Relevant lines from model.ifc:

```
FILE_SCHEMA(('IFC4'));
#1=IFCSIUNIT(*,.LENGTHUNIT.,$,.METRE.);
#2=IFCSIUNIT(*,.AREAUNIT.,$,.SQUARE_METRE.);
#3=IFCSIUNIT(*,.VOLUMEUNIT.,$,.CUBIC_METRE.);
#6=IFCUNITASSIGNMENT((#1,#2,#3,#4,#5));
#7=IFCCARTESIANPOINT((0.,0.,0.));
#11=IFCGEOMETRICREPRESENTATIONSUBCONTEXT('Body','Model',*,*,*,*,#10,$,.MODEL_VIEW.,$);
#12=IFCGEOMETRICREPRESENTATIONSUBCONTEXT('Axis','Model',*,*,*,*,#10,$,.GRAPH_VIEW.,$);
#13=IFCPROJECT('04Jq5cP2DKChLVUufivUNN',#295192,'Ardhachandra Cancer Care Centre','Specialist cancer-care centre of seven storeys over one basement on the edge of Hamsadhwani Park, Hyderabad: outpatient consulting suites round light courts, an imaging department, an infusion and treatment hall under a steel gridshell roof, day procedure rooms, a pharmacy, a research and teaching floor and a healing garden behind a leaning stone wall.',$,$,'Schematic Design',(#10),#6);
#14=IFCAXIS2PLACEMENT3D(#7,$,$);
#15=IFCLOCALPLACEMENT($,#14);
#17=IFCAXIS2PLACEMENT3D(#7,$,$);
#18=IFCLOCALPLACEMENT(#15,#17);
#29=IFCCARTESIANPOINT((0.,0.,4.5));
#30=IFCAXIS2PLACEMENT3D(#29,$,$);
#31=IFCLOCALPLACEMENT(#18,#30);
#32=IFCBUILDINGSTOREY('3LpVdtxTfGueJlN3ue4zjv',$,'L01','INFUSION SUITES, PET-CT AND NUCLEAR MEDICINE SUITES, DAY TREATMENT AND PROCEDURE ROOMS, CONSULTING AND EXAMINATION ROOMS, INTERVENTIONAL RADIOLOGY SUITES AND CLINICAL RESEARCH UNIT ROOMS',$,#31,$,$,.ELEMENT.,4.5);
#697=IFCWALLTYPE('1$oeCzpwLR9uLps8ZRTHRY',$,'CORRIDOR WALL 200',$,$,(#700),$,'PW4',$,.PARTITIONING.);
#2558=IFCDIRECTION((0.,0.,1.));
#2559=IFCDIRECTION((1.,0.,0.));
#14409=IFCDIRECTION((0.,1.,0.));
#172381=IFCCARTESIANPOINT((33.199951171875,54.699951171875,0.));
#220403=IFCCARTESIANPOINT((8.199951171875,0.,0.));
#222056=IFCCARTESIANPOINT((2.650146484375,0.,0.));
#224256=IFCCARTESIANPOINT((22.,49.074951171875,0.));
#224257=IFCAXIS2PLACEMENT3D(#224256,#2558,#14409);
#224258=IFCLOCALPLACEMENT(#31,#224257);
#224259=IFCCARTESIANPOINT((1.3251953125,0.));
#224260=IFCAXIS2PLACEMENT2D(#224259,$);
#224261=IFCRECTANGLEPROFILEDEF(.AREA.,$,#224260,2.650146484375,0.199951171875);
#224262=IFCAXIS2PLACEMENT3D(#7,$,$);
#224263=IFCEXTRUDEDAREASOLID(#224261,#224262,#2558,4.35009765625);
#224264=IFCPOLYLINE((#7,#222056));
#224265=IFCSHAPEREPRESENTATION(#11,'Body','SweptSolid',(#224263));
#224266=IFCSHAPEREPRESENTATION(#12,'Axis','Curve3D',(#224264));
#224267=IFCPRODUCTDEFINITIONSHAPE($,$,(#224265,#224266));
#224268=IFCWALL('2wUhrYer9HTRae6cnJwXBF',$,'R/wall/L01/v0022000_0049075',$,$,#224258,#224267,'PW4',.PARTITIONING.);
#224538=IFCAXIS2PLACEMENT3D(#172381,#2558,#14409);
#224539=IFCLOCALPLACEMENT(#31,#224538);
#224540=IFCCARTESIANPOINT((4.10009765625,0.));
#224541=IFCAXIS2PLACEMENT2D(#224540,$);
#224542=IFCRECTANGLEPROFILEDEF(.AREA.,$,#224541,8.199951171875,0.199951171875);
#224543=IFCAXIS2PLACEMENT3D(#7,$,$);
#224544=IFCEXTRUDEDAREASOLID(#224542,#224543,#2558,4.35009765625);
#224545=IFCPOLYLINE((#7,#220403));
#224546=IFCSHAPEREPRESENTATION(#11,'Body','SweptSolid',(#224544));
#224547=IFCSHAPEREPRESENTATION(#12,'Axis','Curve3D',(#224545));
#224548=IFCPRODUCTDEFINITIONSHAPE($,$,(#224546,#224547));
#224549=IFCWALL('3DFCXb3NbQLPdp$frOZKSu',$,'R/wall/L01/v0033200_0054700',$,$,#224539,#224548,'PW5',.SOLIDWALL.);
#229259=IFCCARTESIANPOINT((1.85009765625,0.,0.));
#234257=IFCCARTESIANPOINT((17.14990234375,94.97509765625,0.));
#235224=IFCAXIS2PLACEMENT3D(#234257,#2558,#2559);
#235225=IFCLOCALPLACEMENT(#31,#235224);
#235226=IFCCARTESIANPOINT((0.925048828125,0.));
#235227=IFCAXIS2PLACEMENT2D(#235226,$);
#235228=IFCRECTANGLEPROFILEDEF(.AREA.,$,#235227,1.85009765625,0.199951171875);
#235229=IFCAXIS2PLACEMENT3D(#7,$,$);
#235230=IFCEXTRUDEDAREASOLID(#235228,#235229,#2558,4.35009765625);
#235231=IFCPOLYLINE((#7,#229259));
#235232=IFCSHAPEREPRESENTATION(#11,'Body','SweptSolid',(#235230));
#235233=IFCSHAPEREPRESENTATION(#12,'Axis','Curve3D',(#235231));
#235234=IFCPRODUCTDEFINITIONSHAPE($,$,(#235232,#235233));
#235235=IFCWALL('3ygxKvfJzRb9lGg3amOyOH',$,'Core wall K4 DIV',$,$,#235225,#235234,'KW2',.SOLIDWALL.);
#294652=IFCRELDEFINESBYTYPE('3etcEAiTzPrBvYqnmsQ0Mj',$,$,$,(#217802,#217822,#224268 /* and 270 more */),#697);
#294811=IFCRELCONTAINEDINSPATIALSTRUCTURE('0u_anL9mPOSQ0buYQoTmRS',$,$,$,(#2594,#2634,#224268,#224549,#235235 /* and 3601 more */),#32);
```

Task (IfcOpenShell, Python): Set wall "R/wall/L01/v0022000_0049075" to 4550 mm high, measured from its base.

```python
import ifcopenshell
import ifcopenshell.geom
import ifcopenshell.util.representation
import ifcopenshell.util.shape
import ifcopenshell.util.unit

model = ifcopenshell.open("model.ifc")
unit_scale = ifcopenshell.util.unit.calculate_unit_scale(model)
settings = ifcopenshell.geom.settings()


def volume(element):
    """Net volume in cubic metres, openings subtracted."""
    shape = ifcopenshell.geom.create_shape(settings, element)
    return ifcopenshell.util.shape.get_volume(shape.geometry)


wall = model.by_guid("2wUhrYer9HTRae6cnJwXBF")
before = volume(wall)

body = ifcopenshell.util.representation.get_representation(wall, "Model", "Body")
solid = body.Items[0]
old_height = solid.Depth
solid.Depth = 4.55 / unit_scale
after = volume(wall)

print(f"height {old_height:g} -> {solid.Depth:g}, volume {before:.3f} -> {after:.3f} m3")

model.write("model_updated.ifc")
```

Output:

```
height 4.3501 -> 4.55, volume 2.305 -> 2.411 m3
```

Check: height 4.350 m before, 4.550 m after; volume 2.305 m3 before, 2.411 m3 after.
